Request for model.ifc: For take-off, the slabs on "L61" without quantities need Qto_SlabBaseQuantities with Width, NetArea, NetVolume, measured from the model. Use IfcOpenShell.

First a look at what the model holds.

```python
import ifcopenshell
import ifcopenshell.util.element
import ifcopenshell.util.unit

model = ifcopenshell.open("model.ifc")
print(model.schema)
for unit_type in ("LENGTHUNIT", "AREAUNIT", "VOLUMEUNIT"):
    print(unit_type, ifcopenshell.util.unit.calculate_unit_scale(model, unit_type))
storey = next(s for s in model.by_type("IfcBuildingStorey") if s.Name == "L61")
slabs = [e for e in ifcopenshell.util.element.get_decomposition(storey) if e.is_a("IfcSlab")]
for e in sorted(slabs, key=lambda e: e.id()):
    print(e.id(), e.is_a(), e.Name, list(ifcopenshell.util.element.get_psets(e, qtos_only=True)), sep=" | ")
```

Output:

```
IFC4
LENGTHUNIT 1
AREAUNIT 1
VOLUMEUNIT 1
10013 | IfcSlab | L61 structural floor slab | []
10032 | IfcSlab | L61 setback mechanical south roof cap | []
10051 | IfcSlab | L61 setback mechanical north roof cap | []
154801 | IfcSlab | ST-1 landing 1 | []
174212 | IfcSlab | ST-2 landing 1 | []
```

```python
import ifcopenshell
import ifcopenshell.api.pset
import ifcopenshell.geom
import ifcopenshell.util.element
import ifcopenshell.util.shape
import ifcopenshell.util.unit

model = ifcopenshell.open("model.ifc")
unit_scale = ifcopenshell.util.unit.calculate_unit_scale(model)
area_scale = ifcopenshell.util.unit.calculate_unit_scale(model, "AREAUNIT")
volume_scale = ifcopenshell.util.unit.calculate_unit_scale(model, "VOLUMEUNIT")
settings = ifcopenshell.geom.settings()

storey = next(s for s in model.by_type("IfcBuildingStorey") if s.Name == "L61")
slabs = [e for e in ifcopenshell.util.element.get_decomposition(storey) if e.is_a("IfcSlab")]

for e in sorted(slabs, key=lambda e: e.id()):
    if ifcopenshell.util.element.get_psets(e, qtos_only=True, should_inherit=False):
        continue
    # Geometry comes back in metres, in the element's own axes.
    shape = ifcopenshell.geom.create_shape(settings, e)
    values = {
        "Width": ifcopenshell.util.shape.get_z(shape.geometry) / unit_scale,
        "NetArea": ifcopenshell.util.shape.get_footprint_area(shape.geometry) / area_scale,
        "NetVolume": ifcopenshell.util.shape.get_volume(shape.geometry) / volume_scale,
    }
    qto = ifcopenshell.api.pset.add_qto(model, product=e, name="Qto_SlabBaseQuantities")
    ifcopenshell.api.pset.edit_qto(model, qto=qto, properties=values)
    print(e.id(), {k: round(v, 3) for k, v in values.items()})

model.write("model-out.ifc")
```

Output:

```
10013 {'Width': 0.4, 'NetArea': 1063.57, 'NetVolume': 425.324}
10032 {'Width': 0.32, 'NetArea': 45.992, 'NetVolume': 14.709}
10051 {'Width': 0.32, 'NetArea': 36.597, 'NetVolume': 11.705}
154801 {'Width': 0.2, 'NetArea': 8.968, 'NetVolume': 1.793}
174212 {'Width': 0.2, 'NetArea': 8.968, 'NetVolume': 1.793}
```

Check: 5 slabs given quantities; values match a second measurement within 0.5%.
